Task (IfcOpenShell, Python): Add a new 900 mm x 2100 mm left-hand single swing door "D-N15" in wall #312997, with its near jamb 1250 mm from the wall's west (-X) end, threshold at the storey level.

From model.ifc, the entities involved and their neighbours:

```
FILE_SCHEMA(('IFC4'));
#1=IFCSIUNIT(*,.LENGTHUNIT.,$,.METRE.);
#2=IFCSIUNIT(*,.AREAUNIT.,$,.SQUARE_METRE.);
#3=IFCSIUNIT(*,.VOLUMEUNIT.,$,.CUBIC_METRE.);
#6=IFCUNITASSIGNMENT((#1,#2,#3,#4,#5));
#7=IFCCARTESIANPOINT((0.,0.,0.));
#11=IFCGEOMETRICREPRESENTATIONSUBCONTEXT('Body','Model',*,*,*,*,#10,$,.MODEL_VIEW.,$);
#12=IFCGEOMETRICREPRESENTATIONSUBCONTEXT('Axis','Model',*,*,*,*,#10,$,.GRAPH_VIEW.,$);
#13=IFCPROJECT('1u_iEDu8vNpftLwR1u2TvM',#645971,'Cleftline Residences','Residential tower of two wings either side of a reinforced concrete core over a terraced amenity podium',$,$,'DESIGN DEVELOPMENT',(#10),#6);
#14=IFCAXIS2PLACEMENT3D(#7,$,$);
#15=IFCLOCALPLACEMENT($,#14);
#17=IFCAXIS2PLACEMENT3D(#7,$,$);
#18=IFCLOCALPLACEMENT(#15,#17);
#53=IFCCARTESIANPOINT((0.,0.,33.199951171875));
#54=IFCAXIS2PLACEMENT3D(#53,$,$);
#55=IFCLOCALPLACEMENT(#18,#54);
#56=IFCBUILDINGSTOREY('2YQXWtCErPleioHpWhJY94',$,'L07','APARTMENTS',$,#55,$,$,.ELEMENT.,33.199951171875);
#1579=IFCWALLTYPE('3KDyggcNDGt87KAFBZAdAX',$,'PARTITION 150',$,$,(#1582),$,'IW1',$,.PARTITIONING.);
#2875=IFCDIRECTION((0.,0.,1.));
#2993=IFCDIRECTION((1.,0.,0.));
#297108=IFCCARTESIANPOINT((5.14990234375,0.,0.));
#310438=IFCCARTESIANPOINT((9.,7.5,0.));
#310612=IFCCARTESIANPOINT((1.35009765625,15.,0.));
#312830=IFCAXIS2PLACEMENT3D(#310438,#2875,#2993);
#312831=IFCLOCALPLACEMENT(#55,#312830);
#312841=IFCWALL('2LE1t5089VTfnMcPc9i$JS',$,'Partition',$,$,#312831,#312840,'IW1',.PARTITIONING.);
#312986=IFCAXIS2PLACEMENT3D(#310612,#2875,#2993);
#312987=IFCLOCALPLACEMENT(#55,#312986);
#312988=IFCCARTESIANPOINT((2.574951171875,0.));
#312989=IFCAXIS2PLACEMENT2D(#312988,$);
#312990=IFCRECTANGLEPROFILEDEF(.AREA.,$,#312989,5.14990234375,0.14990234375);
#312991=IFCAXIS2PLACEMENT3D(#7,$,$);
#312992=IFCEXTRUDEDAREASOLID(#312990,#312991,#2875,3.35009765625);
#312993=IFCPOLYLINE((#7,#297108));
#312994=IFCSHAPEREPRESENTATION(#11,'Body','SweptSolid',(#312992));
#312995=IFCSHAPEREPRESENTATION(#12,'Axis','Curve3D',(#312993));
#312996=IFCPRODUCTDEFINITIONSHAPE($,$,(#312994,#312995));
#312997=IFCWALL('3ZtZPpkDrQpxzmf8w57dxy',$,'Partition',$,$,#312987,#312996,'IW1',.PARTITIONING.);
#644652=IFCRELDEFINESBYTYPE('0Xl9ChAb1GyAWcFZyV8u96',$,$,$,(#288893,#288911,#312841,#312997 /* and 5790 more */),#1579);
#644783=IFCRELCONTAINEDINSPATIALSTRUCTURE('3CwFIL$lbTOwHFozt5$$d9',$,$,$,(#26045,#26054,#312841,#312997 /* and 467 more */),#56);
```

```python
import numpy as np
import ifcopenshell
import ifcopenshell.api.feature
import ifcopenshell.api.geometry
import ifcopenshell.api.root
import ifcopenshell.api.spatial
import ifcopenshell.geom
import ifcopenshell.util.element
import ifcopenshell.util.placement
import ifcopenshell.util.representation
import ifcopenshell.util.shape
import ifcopenshell.util.unit

model = ifcopenshell.open("model.ifc")
unit_scale = ifcopenshell.util.unit.calculate_unit_scale(model)
settings = ifcopenshell.geom.settings()


def volume(element):
    """Net volume in cubic metres, openings subtracted."""
    shape = ifcopenshell.geom.create_shape(settings, element)
    return ifcopenshell.util.shape.get_volume(shape.geometry)


wall = model.by_id(312997)
storey = ifcopenshell.util.element.get_container(wall, ifc_class="IfcBuildingStorey")
context = ifcopenshell.util.representation.get_context(model, "Model", "Body", "MODEL_VIEW")
before = volume(wall)

width, height, from_end, sill = 0.9, 2.1, 1.25, 0.0  # metres

# The wall runs along its own X axis, and the end named is its -X end.
wall_shape = ifcopenshell.geom.create_shape(settings, wall)
x, y, z = ifcopenshell.util.shape.get_vertices(wall_shape.geometry).T
start = x.min() + from_end
face, thickness = float(y.min()), float(y.max() - y.min())
wall_matrix = ifcopenshell.util.placement.get_local_placement(wall.ObjectPlacement)
level = ifcopenshell.util.placement.get_local_placement(storey.ObjectPlacement)[2, 3]


def in_wall(x, y):
    """Placement at x, y metres in the wall's axes, at sill height."""
    matrix = wall_matrix.copy()
    matrix[:, 3] = wall_matrix @ np.array([x / unit_scale, y / unit_scale, 0.0, 1.0])
    matrix[2, 3] = level + sill / unit_scale
    return matrix


# Opening: a box that overshoots both wall faces by 50 mm.
opening = ifcopenshell.api.root.create_entity(model, ifc_class="IfcOpeningElement", predefined_type="OPENING")
box = ifcopenshell.api.geometry.add_wall_representation(
    model, context=context, length=width, height=height, thickness=thickness + 0.1
)
ifcopenshell.api.geometry.assign_representation(model, product=opening, representation=box)
ifcopenshell.api.geometry.edit_object_placement(model, product=opening, matrix=in_wall(start, face - 0.05), is_si=False)
ifcopenshell.api.feature.add_feature(model, feature=opening, element=wall)

door = ifcopenshell.api.root.create_entity(model, ifc_class="IfcDoor", name="D-N15", predefined_type="DOOR")
door.OverallWidth, door.OverallHeight = width / unit_scale, height / unit_scale
door.OperationType = "SINGLE_SWING_LEFT"
body = ifcopenshell.api.geometry.add_door_representation(
    model,
    context=context,
    overall_width=door.OverallWidth,
    overall_height=door.OverallHeight,
    operation_type="SINGLE_SWING_LEFT",
    lining_properties={"LiningDepth": thickness / unit_scale, "ThresholdDepth": thickness / unit_scale},
)
ifcopenshell.api.geometry.assign_representation(model, product=door, representation=body)
ifcopenshell.api.spatial.assign_container(model, products=[door], relating_structure=storey)
ifcopenshell.api.feature.add_filling(model, opening=opening, element=door)

# The lining spans the wall, so the door starts at the wall face.
ifcopenshell.api.geometry.edit_object_placement(model, product=door, matrix=in_wall(start, face), is_si=False)

after = volume(wall)

print(f"wall volume {before:.3f} -> {after:.3f} m3")

model.write("model_v2.ifc")
```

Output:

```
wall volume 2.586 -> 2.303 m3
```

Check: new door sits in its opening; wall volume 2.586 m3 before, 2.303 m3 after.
